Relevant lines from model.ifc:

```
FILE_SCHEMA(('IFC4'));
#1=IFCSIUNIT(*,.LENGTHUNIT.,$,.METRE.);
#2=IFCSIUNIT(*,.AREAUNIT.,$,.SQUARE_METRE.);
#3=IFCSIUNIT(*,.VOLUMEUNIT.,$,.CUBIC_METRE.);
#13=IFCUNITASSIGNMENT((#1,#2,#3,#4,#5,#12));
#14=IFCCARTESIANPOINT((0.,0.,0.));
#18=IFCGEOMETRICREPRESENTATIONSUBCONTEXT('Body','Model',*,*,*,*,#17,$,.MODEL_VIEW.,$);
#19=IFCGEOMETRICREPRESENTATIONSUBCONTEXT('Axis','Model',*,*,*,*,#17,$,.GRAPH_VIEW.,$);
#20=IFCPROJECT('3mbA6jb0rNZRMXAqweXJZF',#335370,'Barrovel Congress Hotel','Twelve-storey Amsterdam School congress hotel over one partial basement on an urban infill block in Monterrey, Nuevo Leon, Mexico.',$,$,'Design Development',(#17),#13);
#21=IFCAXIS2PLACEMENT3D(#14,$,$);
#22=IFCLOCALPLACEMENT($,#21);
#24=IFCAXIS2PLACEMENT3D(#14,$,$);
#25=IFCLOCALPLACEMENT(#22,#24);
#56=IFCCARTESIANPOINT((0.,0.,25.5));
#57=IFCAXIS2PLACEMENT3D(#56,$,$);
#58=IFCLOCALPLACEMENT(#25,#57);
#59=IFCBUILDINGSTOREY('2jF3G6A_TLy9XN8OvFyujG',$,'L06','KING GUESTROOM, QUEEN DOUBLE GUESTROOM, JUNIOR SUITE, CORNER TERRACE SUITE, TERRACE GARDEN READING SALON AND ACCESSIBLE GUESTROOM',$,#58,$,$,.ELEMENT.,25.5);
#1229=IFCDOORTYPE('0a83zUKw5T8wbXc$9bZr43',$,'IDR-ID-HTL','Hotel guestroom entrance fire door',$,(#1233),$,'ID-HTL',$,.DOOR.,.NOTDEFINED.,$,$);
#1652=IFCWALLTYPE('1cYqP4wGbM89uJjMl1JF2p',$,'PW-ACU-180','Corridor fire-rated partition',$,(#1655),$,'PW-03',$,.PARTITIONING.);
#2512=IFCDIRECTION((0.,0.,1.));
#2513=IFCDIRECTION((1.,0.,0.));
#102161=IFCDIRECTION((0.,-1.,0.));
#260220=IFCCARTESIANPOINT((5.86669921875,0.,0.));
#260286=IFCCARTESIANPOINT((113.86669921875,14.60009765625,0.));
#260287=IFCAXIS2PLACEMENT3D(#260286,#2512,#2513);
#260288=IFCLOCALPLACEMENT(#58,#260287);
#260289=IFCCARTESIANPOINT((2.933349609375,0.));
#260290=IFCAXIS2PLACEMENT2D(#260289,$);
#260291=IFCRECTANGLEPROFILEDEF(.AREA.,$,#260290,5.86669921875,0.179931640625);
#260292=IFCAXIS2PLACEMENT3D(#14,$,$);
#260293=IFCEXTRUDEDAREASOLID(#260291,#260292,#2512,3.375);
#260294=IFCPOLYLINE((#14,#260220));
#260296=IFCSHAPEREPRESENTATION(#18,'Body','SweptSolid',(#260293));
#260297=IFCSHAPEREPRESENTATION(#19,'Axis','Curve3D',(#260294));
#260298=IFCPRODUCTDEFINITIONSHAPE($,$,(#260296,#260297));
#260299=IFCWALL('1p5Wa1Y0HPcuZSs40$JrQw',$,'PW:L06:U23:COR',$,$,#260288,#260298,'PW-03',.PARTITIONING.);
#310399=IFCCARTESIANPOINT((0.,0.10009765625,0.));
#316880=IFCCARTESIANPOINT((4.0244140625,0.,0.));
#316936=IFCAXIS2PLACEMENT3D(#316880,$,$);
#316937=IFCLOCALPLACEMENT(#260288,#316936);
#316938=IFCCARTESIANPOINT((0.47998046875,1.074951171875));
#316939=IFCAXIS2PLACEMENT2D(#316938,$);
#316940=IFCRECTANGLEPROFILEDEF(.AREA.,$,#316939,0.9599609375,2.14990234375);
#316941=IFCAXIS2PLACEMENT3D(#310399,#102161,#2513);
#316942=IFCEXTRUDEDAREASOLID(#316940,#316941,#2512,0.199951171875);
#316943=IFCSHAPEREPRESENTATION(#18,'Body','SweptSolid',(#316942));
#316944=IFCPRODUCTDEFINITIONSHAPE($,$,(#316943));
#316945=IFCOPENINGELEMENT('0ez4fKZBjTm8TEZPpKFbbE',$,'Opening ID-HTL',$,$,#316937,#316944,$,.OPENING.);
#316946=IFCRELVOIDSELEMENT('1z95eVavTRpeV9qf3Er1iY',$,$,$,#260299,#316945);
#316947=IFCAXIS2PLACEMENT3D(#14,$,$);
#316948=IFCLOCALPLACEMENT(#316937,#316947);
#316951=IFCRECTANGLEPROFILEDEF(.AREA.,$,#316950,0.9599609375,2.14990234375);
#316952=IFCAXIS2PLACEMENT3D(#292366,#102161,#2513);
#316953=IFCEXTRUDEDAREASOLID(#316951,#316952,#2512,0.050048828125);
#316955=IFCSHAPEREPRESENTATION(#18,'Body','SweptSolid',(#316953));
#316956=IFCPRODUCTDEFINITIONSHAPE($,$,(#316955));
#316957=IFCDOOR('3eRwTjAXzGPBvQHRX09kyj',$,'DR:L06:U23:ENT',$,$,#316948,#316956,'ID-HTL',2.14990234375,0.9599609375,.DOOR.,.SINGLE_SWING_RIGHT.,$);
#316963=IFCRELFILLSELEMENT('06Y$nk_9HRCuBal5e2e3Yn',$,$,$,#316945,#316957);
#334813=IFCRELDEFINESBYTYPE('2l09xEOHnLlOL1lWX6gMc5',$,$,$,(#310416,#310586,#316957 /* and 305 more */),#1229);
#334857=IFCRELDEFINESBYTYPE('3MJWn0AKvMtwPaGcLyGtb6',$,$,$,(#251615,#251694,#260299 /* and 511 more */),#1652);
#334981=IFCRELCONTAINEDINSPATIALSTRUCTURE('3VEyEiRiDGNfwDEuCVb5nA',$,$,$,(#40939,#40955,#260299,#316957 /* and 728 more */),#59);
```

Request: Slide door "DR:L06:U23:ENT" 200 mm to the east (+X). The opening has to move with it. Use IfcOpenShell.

```python
import ifcopenshell
import ifcopenshell.api.geometry
import ifcopenshell.util.placement

model = ifcopenshell.open("model.ifc")

door = model.by_guid("3eRwTjAXzGPBvQHRX09kyj")
opening = door.FillsVoids[0].RelatingOpeningElement
wall = opening.VoidsElements[0].RelatingBuildingElement

wall_matrix = ifcopenshell.util.placement.get_local_placement(wall.ObjectPlacement)
shift = wall_matrix[:3, 0] * 0.2
before = ifcopenshell.util.placement.get_local_placement(door.ObjectPlacement)[:3, 3].copy()

# The door is placed relative to its opening, so it follows when the opening moves.
matrix = ifcopenshell.util.placement.get_local_placement(opening.ObjectPlacement)
matrix[:3, 3] += shift
ifcopenshell.api.geometry.edit_object_placement(
    model, product=opening, matrix=matrix, is_si=False, should_transform_children=True
)

after = ifcopenshell.util.placement.get_local_placement(door.ObjectPlacement)[:3, 3]
print("door moved by", (after - before).round(3) + 0.0)

model.write("model-out.ifc")
```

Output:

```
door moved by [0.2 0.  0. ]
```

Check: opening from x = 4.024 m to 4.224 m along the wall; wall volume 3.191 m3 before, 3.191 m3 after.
